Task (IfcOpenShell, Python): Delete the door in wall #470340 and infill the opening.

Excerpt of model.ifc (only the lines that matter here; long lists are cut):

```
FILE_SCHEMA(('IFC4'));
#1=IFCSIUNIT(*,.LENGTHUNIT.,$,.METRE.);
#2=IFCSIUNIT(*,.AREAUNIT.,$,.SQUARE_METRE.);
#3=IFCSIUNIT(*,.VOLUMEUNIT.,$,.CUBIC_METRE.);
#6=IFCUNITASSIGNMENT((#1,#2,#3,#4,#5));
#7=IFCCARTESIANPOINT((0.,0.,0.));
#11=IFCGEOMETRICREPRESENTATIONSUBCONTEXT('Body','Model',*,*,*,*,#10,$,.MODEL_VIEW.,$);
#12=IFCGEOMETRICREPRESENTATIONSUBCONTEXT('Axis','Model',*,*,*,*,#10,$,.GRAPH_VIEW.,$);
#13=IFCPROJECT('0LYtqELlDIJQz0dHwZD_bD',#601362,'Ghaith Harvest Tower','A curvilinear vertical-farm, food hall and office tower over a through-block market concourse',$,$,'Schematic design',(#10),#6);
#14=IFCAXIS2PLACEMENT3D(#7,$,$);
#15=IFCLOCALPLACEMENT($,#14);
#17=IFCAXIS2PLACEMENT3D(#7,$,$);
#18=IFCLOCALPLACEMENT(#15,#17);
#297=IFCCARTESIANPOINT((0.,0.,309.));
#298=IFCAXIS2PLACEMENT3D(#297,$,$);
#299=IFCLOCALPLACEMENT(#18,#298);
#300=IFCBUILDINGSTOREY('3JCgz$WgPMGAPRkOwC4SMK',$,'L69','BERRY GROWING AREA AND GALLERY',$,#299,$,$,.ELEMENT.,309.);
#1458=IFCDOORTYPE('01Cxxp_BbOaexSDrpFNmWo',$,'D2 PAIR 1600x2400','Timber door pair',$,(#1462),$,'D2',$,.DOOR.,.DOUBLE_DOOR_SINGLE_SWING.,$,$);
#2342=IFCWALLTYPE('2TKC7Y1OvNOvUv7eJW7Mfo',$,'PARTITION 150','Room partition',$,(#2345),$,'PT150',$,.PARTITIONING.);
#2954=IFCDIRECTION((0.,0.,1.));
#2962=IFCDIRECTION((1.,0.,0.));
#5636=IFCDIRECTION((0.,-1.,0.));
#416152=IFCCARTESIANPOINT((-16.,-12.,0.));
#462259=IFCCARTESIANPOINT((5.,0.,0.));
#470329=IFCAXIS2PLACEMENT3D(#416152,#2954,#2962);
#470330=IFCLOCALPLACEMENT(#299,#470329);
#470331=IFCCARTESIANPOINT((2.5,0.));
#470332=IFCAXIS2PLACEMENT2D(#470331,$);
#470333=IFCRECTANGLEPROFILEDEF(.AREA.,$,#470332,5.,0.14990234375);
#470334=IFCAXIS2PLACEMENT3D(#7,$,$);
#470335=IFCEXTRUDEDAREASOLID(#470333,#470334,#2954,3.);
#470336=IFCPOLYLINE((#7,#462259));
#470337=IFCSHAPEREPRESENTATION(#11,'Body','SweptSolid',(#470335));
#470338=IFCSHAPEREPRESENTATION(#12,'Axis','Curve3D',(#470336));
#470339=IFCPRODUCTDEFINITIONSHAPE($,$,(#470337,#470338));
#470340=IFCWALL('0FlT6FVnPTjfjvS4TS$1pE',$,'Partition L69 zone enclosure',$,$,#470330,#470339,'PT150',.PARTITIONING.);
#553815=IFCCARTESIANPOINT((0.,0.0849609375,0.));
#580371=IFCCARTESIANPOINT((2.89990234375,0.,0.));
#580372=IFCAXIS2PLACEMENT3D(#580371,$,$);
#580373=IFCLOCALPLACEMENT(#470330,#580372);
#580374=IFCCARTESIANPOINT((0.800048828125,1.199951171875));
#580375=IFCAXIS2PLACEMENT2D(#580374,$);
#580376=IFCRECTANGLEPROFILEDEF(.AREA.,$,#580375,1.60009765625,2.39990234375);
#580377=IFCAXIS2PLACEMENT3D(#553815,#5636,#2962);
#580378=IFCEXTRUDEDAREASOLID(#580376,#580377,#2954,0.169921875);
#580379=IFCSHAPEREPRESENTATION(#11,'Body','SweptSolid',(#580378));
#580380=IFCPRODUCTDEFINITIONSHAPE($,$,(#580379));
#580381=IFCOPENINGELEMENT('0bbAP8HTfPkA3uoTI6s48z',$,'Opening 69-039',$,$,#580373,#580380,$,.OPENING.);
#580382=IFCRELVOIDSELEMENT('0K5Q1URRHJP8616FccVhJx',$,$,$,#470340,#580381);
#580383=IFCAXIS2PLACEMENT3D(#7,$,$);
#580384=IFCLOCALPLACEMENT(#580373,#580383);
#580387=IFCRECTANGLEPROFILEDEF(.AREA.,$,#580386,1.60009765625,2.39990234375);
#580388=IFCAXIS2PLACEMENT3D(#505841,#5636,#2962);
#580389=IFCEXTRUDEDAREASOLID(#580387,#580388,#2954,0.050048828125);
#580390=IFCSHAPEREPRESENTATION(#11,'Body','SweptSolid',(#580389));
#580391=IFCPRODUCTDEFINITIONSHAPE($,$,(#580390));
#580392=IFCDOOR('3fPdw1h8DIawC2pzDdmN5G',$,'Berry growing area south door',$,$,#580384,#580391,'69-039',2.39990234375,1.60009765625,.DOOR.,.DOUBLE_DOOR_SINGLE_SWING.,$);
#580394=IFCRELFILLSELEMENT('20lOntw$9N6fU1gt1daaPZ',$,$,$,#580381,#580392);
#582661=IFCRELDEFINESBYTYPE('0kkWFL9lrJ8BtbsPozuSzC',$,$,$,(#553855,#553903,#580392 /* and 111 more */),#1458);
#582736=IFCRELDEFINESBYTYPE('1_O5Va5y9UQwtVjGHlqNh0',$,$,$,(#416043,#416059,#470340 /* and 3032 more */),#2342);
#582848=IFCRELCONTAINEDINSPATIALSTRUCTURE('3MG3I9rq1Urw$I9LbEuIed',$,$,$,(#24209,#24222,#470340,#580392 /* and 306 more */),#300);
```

```python
import ifcopenshell
import ifcopenshell.api.feature
import ifcopenshell.api.root
import ifcopenshell.geom
import ifcopenshell.util.shape

model = ifcopenshell.open("model.ifc")
settings = ifcopenshell.geom.settings()


def volume(element):
    """Net volume in cubic metres, openings subtracted."""
    shape = ifcopenshell.geom.create_shape(settings, element)
    return ifcopenshell.util.shape.get_volume(shape.geometry)


door = model.by_id(580392)
opening = door.FillsVoids[0].RelatingOpeningElement
wall = opening.VoidsElements[0].RelatingBuildingElement
before = volume(wall)

ifcopenshell.api.root.remove_product(model, product=door)
ifcopenshell.api.feature.remove_feature(model, feature=opening)

after = volume(wall)

print(f"wall volume {before:.3f} -> {after:.3f} m3")

model.write("model_rev.ifc")
```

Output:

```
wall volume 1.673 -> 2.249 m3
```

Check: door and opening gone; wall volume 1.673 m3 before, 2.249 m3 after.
